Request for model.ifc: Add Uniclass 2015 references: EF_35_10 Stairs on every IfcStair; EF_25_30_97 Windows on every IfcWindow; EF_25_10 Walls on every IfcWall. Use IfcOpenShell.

First a look at what the model holds.

```python
import ifcopenshell

model = ifcopenshell.open("model.ifc")
print(model.schema)
print("classifications:", [c.Name for c in model.by_type("IfcClassification")])
for ifc_class in ("IfcDoor", "IfcRoof", "IfcStair", "IfcWall", "IfcWindow"):
    print(ifc_class, len(model.by_type(ifc_class)))
```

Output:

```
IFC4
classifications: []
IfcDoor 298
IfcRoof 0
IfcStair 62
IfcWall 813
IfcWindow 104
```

```python
import ifcopenshell
import ifcopenshell.api.classification

model = ifcopenshell.open("model.ifc")

system = ifcopenshell.api.classification.add_classification(model, classification="Uniclass 2015")

codes = {
    "IfcStair": ("EF_35_10", "Stairs"),
    "IfcWindow": ("EF_25_30_97", "Windows"),
    "IfcWall": ("EF_25_10", "Walls"),
}
for ifc_class, (code, name) in codes.items():
    products = model.by_type(ifc_class)
    ifcopenshell.api.classification.add_reference(
        model, products=products, classification=system, identification=code, name=name
    )
    print(code, len(products))

model.write("model_rev.ifc")
```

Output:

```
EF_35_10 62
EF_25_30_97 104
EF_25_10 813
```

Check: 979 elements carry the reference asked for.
